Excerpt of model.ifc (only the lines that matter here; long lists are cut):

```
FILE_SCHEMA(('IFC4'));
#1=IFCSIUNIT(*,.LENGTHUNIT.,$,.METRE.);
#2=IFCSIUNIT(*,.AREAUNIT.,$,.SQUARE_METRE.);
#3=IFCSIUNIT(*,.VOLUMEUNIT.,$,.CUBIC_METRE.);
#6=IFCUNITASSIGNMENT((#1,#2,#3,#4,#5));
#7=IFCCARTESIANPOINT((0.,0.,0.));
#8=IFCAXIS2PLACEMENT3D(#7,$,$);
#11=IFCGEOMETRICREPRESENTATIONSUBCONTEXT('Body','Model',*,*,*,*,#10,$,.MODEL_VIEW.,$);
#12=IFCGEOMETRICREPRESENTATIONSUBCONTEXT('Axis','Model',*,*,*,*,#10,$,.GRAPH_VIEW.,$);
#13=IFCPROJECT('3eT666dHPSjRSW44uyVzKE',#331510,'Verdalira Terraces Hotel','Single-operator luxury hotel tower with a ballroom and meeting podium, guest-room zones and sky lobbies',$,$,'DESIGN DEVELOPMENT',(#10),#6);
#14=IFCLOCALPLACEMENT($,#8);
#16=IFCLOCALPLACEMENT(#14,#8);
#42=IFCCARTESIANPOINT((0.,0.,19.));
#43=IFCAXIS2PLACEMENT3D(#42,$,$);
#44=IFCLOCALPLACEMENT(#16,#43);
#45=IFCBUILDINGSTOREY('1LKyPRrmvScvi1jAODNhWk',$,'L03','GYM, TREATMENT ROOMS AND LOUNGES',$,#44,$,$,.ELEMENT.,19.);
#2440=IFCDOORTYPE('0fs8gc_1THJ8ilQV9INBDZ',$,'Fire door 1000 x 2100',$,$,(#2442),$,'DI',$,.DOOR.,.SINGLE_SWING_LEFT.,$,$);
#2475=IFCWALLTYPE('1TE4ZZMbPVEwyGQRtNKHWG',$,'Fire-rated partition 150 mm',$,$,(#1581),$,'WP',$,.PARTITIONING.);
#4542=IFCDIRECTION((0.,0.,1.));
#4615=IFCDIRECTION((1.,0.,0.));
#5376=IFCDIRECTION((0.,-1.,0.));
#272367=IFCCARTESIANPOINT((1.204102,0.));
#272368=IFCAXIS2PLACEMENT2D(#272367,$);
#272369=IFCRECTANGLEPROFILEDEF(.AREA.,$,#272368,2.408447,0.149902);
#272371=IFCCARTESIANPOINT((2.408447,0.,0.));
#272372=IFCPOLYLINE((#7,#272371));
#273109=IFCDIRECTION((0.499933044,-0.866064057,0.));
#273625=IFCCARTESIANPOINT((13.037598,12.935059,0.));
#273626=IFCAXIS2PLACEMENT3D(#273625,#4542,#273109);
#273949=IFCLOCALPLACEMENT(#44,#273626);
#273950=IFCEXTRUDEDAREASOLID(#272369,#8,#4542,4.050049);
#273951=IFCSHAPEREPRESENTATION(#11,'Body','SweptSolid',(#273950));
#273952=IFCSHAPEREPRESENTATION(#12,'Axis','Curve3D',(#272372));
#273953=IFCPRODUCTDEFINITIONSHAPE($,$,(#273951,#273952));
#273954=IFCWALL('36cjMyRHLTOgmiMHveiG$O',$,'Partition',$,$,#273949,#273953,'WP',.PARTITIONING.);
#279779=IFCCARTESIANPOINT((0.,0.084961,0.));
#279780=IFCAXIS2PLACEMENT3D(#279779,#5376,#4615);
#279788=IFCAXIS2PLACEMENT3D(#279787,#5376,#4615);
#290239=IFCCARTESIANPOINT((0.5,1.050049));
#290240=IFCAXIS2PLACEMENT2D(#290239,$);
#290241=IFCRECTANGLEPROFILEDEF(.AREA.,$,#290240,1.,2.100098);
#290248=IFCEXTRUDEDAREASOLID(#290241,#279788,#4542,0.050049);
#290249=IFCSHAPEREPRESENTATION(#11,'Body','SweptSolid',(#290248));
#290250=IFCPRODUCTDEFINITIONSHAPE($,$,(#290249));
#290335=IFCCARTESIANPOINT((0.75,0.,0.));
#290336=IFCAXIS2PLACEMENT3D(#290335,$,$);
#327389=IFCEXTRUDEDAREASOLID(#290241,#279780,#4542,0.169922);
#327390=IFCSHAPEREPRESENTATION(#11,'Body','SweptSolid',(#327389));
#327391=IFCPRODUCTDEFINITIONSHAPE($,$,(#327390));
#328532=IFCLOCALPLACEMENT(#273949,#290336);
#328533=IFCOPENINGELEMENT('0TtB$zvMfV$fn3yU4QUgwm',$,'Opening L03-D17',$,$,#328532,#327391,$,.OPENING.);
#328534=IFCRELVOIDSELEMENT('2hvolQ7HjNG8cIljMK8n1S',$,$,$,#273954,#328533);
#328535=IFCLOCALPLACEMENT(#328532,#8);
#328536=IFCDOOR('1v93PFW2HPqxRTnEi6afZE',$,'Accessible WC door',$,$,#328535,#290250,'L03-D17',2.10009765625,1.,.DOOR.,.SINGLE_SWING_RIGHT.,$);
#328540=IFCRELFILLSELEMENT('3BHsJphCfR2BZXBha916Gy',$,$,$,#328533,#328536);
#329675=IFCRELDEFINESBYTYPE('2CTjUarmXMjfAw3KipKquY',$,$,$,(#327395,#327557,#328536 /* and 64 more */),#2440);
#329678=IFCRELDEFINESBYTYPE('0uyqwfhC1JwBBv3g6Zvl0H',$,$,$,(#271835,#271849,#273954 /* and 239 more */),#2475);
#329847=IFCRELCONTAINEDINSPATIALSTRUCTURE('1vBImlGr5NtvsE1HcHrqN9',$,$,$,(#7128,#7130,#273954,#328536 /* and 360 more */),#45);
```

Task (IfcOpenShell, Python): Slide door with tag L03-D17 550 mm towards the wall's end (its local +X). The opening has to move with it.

```python
import ifcopenshell
import ifcopenshell.api.geometry
import ifcopenshell.util.placement

model = ifcopenshell.open("model.ifc")

door = model.by_guid("1v93PFW2HPqxRTnEi6afZE")
opening = door.FillsVoids[0].RelatingOpeningElement
wall = opening.VoidsElements[0].RelatingBuildingElement

wall_matrix = ifcopenshell.util.placement.get_local_placement(wall.ObjectPlacement)
shift = wall_matrix[:3, 0] * 0.55
before = ifcopenshell.util.placement.get_local_placement(door.ObjectPlacement)[:3, 3].copy()

# The door is placed relative to its opening, so it follows when the opening moves.
matrix = ifcopenshell.util.placement.get_local_placement(opening.ObjectPlacement)
matrix[:3, 3] += shift
ifcopenshell.api.geometry.edit_object_placement(
    model, product=opening, matrix=matrix, is_si=False, should_transform_children=True
)

after = ifcopenshell.util.placement.get_local_placement(door.ObjectPlacement)[:3, 3]
print("door moved by", (after - before).round(3) + 0.0)

model.write("model_v2.ifc")
```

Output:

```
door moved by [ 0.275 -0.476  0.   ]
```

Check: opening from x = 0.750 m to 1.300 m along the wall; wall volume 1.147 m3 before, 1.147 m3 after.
